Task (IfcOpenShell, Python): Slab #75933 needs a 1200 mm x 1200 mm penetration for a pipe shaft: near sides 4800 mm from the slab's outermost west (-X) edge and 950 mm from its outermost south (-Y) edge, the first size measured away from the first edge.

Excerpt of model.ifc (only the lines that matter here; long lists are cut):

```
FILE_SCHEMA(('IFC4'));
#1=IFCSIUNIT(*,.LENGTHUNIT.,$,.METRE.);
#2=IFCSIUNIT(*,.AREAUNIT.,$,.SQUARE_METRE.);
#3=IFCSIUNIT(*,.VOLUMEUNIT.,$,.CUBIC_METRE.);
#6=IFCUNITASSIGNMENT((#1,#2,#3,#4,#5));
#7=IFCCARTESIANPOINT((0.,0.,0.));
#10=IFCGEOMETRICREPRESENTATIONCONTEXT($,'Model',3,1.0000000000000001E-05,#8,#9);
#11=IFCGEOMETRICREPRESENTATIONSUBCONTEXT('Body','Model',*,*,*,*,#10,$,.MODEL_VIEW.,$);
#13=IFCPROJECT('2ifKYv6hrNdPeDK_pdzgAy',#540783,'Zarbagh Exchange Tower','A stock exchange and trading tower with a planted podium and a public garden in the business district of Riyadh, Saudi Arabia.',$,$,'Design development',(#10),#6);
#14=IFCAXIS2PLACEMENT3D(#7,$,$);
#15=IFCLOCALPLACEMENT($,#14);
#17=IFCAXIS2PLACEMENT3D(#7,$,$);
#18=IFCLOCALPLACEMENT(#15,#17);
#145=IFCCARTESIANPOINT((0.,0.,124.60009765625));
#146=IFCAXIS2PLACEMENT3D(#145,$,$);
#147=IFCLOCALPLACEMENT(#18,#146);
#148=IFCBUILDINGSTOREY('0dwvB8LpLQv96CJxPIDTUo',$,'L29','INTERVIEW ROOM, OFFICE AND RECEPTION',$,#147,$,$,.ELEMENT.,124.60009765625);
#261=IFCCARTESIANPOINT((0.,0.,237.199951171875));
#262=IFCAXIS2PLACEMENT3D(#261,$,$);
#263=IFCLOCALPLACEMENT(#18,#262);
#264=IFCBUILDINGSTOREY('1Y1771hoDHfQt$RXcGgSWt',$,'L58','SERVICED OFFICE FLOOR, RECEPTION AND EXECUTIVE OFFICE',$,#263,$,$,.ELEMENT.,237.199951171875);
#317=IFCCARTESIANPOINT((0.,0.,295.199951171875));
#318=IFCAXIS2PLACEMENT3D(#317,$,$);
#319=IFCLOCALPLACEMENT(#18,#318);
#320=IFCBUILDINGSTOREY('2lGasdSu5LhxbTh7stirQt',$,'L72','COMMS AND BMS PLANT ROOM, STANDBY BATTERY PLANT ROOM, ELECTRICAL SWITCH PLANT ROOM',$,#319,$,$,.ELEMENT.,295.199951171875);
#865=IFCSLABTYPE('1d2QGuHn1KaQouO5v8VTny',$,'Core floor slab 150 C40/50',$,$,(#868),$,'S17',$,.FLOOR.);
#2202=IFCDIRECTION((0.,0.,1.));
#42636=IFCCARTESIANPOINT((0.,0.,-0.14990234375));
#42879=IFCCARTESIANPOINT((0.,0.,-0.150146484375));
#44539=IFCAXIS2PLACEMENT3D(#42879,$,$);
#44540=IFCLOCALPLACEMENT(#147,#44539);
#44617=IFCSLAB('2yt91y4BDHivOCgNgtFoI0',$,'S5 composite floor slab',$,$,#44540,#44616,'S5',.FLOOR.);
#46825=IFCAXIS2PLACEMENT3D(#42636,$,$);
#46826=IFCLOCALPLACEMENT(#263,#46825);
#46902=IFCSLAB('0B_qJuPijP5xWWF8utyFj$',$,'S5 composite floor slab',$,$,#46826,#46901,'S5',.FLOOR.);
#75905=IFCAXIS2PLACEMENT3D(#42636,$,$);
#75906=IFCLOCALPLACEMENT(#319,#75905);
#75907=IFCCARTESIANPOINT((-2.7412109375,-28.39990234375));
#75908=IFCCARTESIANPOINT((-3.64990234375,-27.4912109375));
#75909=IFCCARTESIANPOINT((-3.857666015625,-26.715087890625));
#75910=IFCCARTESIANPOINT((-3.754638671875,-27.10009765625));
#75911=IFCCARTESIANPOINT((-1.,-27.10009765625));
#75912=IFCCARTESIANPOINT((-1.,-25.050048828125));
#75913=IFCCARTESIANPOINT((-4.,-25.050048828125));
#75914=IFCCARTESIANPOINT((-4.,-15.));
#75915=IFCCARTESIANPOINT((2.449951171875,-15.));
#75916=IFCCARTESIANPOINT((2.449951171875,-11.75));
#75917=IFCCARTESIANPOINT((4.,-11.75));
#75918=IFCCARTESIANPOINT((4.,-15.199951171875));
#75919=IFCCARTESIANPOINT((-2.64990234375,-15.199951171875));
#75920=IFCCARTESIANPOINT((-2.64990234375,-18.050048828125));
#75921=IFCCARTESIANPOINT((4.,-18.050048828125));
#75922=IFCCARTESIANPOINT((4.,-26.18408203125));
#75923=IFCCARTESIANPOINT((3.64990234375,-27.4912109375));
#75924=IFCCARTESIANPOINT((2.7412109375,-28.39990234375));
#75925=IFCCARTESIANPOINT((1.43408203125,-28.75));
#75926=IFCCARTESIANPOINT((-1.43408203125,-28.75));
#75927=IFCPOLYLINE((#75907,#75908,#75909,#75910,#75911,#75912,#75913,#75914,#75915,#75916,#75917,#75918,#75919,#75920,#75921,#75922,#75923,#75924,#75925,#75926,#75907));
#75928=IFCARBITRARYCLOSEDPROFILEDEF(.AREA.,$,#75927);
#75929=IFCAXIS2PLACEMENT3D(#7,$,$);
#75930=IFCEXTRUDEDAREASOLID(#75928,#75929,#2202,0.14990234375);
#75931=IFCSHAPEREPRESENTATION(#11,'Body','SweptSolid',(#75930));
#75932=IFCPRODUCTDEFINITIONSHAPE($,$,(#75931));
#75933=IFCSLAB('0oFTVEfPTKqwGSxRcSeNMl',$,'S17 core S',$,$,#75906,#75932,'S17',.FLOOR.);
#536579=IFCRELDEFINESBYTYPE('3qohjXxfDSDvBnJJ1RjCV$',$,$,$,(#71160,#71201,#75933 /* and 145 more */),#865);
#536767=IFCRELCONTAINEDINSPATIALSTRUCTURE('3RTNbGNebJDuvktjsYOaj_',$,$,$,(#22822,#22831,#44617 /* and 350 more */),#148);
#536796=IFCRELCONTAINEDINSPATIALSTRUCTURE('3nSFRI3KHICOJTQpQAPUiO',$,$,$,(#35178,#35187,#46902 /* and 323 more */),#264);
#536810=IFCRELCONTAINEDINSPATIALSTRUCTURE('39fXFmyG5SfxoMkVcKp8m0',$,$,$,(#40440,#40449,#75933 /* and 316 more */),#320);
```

```python
import numpy as np
import ifcopenshell
import ifcopenshell.api.feature
import ifcopenshell.api.geometry
import ifcopenshell.api.root
import ifcopenshell.geom
import ifcopenshell.util.placement
import ifcopenshell.util.representation
import ifcopenshell.util.shape
import ifcopenshell.util.unit

model = ifcopenshell.open("model.ifc")
unit_scale = ifcopenshell.util.unit.calculate_unit_scale(model)
settings = ifcopenshell.geom.settings()


def volume(element):
    """Net volume in cubic metres, openings subtracted."""
    shape = ifcopenshell.geom.create_shape(settings, element)
    return ifcopenshell.util.shape.get_volume(shape.geometry)


slab = model.by_guid("0oFTVEfPTKqwGSxRcSeNMl")
before = volume(slab)

# Extent in the slab's own axes, in metres. The edges named are its -X and -Y sides.
slab_shape = ifcopenshell.geom.create_shape(settings, slab)
vertices = ifcopenshell.util.shape.get_vertices(slab_shape.geometry)
x_min, y_min, bottom = vertices.min(axis=0)
top = vertices[:, 2].max()

opening = ifcopenshell.api.root.create_entity(model, ifc_class="IfcOpeningElement", name="Pipe shaft opening", predefined_type="OPENING")
context = ifcopenshell.util.representation.get_context(model, "Model", "Body", "MODEL_VIEW")
width, depth = 1.2, 1.2
outline = [(0.0, 0.0), (width, 0.0), (width, depth), (0.0, depth), (0.0, 0.0)]
# Overshoot both faces by 50 mm so the cut is clean.
shape = ifcopenshell.api.geometry.add_slab_representation(
    model, context=context, depth=top - bottom + 0.1, polyline=outline
)
ifcopenshell.api.geometry.assign_representation(model, product=opening, representation=shape)

matrix = ifcopenshell.util.placement.get_local_placement(slab.ObjectPlacement)
matrix[:, 3] = matrix @ np.append(np.array([x_min + 4.8, y_min + 0.95, bottom - 0.05]) / unit_scale, 1.0)
ifcopenshell.api.geometry.edit_object_placement(model, product=opening, matrix=matrix, is_si=False)
ifcopenshell.api.feature.add_feature(model, feature=opening, element=slab)

after = volume(slab)

print(f"slab volume {before:.3f} -> {after:.3f} m3")

model.write("model_updated.ifc")
```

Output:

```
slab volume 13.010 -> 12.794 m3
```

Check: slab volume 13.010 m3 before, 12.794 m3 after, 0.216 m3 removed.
